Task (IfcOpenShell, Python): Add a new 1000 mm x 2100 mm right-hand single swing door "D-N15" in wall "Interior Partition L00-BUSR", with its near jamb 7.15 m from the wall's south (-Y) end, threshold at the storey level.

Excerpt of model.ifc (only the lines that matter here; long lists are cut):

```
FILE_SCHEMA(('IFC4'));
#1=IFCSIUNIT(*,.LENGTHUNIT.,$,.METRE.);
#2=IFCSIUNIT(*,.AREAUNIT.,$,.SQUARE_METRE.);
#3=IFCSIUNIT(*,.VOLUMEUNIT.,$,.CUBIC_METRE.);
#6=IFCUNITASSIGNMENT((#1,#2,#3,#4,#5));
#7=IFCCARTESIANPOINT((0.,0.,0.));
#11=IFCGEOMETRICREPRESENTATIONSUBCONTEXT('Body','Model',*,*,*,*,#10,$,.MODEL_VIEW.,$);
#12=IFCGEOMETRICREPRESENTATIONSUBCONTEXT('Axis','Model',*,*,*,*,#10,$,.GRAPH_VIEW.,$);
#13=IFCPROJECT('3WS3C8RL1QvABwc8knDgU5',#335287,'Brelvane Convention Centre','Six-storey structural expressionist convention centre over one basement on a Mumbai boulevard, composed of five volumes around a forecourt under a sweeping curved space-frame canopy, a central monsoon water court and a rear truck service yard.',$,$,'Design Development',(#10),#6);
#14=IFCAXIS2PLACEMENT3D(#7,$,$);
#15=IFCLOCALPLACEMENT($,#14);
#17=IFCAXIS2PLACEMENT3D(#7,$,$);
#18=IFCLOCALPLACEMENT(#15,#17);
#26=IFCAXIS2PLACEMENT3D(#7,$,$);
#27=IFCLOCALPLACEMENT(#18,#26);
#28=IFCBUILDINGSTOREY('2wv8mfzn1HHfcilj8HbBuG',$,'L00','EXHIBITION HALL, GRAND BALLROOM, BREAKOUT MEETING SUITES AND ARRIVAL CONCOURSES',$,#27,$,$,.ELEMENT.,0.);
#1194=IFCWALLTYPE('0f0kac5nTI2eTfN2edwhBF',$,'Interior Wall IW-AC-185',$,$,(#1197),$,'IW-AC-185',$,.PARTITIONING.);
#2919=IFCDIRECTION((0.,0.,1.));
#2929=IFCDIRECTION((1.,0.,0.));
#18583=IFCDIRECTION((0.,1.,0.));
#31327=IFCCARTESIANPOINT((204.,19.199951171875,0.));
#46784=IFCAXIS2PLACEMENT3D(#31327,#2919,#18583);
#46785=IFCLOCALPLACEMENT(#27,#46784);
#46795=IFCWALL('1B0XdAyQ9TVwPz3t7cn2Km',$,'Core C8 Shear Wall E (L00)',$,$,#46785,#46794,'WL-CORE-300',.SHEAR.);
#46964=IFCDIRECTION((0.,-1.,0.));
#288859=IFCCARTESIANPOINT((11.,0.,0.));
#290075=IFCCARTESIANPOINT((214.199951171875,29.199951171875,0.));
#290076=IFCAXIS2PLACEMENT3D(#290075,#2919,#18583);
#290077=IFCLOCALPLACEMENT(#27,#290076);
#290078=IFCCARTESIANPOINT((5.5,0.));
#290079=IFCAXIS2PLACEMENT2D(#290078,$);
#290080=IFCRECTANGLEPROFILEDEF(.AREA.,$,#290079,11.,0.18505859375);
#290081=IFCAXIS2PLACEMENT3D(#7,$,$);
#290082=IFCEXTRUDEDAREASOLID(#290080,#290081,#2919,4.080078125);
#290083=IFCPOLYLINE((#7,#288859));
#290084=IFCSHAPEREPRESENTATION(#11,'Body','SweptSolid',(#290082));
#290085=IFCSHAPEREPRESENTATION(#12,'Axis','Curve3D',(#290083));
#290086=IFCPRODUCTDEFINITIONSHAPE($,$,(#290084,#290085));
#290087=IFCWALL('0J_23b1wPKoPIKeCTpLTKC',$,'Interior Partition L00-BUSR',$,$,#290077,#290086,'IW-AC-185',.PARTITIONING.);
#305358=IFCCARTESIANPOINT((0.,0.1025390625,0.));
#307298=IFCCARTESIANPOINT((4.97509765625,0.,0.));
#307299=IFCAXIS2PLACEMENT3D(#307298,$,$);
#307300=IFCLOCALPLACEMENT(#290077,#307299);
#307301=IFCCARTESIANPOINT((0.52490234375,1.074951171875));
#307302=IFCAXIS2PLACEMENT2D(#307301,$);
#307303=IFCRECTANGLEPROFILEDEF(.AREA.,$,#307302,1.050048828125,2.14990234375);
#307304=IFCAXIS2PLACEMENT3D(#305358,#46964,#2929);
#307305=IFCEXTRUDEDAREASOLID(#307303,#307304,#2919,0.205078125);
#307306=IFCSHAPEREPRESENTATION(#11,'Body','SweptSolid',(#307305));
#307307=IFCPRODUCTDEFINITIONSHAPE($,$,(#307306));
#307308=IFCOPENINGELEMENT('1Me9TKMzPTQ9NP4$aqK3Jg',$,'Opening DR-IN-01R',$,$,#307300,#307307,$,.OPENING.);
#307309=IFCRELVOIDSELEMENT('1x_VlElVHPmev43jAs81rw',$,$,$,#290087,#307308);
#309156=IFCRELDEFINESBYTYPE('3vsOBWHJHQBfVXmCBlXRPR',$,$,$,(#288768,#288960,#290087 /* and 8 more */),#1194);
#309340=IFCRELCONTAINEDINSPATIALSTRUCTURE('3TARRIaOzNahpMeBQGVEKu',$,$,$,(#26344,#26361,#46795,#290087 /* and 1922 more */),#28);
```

```python
import numpy as np
import ifcopenshell
import ifcopenshell.api.feature
import ifcopenshell.api.geometry
import ifcopenshell.api.root
import ifcopenshell.api.spatial
import ifcopenshell.geom
import ifcopenshell.util.element
import ifcopenshell.util.placement
import ifcopenshell.util.representation
import ifcopenshell.util.shape
import ifcopenshell.util.unit

model = ifcopenshell.open("model.ifc")
unit_scale = ifcopenshell.util.unit.calculate_unit_scale(model)
settings = ifcopenshell.geom.settings()


def volume(element):
    """Net volume in cubic metres, openings subtracted."""
    shape = ifcopenshell.geom.create_shape(settings, element)
    return ifcopenshell.util.shape.get_volume(shape.geometry)


wall = model.by_guid("0J_23b1wPKoPIKeCTpLTKC")
storey = ifcopenshell.util.element.get_container(wall, ifc_class="IfcBuildingStorey")
context = ifcopenshell.util.representation.get_context(model, "Model", "Body", "MODEL_VIEW")
before = volume(wall)

width, height, from_end, sill = 1, 2.1, 7.15, 0.0  # metres

# The wall runs along its own X axis, and the end named is its -X end.
wall_shape = ifcopenshell.geom.create_shape(settings, wall)
x, y, z = ifcopenshell.util.shape.get_vertices(wall_shape.geometry).T
start = x.min() + from_end
face, thickness = float(y.min()), float(y.max() - y.min())
wall_matrix = ifcopenshell.util.placement.get_local_placement(wall.ObjectPlacement)
level = ifcopenshell.util.placement.get_local_placement(storey.ObjectPlacement)[2, 3]


def in_wall(x, y):
    """Placement at x, y metres in the wall's axes, at sill height."""
    matrix = wall_matrix.copy()
    matrix[:, 3] = wall_matrix @ np.array([x / unit_scale, y / unit_scale, 0.0, 1.0])
    matrix[2, 3] = level + sill / unit_scale
    return matrix


# Opening: a box that overshoots both wall faces by 50 mm.
opening = ifcopenshell.api.root.create_entity(model, ifc_class="IfcOpeningElement", predefined_type="OPENING")
box = ifcopenshell.api.geometry.add_wall_representation(
    model, context=context, length=width, height=height, thickness=thickness + 0.1
)
ifcopenshell.api.geometry.assign_representation(model, product=opening, representation=box)
ifcopenshell.api.geometry.edit_object_placement(model, product=opening, matrix=in_wall(start, face - 0.05), is_si=False)
ifcopenshell.api.feature.add_feature(model, feature=opening, element=wall)

door = ifcopenshell.api.root.create_entity(model, ifc_class="IfcDoor", name="D-N15", predefined_type="DOOR")
door.OverallWidth, door.OverallHeight = width / unit_scale, height / unit_scale
door.OperationType = "SINGLE_SWING_RIGHT"
body = ifcopenshell.api.geometry.add_door_representation(
    model,
    context=context,
    overall_width=door.OverallWidth,
    overall_height=door.OverallHeight,
    operation_type="SINGLE_SWING_RIGHT",
    lining_properties={"LiningDepth": thickness / unit_scale, "ThresholdDepth": thickness / unit_scale},
)
ifcopenshell.api.geometry.assign_representation(model, product=door, representation=body)
ifcopenshell.api.spatial.assign_container(model, products=[door], relating_structure=storey)
ifcopenshell.api.feature.add_filling(model, opening=opening, element=door)

# The lining spans the wall, so the door starts at the wall face.
ifcopenshell.api.geometry.edit_object_placement(model, product=door, matrix=in_wall(start, face), is_si=False)

after = volume(wall)

print(f"wall volume {before:.3f} -> {after:.3f} m3")

model.write("model-out.ifc")
```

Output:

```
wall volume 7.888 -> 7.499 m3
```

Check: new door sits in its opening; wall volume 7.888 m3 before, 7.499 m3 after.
